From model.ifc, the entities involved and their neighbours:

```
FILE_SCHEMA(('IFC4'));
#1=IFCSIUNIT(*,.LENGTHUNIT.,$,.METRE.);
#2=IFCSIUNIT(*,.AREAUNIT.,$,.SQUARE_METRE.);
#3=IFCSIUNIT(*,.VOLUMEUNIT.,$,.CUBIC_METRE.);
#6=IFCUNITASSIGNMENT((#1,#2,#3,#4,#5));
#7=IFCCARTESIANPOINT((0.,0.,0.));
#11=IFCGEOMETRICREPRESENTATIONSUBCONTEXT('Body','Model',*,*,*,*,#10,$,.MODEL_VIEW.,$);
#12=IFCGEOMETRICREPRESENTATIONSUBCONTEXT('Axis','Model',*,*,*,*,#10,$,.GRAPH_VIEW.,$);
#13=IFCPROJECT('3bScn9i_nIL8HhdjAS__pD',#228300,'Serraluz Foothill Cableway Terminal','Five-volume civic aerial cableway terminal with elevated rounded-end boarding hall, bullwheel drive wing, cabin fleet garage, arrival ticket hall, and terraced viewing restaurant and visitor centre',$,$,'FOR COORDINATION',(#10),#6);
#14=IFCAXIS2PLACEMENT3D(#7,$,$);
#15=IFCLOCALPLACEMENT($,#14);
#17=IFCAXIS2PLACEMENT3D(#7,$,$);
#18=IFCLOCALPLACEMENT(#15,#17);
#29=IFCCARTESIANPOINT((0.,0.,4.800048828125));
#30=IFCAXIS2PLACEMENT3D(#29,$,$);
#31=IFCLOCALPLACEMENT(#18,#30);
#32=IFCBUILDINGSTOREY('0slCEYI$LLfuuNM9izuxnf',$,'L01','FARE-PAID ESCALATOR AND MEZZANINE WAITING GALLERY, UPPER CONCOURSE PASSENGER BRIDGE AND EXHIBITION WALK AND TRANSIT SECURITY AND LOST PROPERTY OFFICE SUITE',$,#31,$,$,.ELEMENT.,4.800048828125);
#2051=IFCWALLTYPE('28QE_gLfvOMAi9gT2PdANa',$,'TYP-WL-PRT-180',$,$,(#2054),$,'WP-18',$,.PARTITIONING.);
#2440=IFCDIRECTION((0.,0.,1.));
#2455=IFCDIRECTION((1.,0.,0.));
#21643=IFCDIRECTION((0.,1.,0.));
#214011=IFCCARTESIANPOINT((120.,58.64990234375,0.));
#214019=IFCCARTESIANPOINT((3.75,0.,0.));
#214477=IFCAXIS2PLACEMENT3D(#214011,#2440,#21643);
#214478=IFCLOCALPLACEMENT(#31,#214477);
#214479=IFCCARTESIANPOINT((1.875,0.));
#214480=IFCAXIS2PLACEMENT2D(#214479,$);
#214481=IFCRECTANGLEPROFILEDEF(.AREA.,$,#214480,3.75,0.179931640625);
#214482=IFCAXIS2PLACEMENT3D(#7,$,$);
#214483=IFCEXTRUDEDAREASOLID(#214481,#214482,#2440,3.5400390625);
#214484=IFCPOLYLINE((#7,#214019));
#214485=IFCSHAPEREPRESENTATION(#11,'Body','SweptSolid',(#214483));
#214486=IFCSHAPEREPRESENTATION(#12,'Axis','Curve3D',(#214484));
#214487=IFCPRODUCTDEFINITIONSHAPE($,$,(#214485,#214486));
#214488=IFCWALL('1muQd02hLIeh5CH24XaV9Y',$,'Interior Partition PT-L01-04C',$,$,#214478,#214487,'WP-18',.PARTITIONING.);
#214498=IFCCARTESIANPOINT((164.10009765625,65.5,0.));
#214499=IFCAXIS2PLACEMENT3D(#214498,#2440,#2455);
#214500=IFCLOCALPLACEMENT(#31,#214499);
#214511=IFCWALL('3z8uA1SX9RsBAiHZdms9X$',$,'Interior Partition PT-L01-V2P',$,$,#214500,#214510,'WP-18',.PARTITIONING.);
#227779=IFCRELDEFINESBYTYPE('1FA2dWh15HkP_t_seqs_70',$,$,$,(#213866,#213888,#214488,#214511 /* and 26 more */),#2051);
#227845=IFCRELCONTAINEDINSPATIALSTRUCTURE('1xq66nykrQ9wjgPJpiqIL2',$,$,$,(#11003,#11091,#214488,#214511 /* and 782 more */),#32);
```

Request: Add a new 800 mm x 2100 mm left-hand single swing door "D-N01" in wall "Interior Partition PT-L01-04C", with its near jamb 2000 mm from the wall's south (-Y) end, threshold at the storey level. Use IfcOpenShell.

```python
import numpy as np
import ifcopenshell
import ifcopenshell.api.feature
import ifcopenshell.api.geometry
import ifcopenshell.api.root
import ifcopenshell.api.spatial
import ifcopenshell.geom
import ifcopenshell.util.element
import ifcopenshell.util.placement
import ifcopenshell.util.representation
import ifcopenshell.util.shape
import ifcopenshell.util.unit

model = ifcopenshell.open("model.ifc")
unit_scale = ifcopenshell.util.unit.calculate_unit_scale(model)
settings = ifcopenshell.geom.settings()


def volume(element):
    """Net volume in cubic metres, openings subtracted."""
    shape = ifcopenshell.geom.create_shape(settings, element)
    return ifcopenshell.util.shape.get_volume(shape.geometry)


wall = model.by_id(214488)
storey = ifcopenshell.util.element.get_container(wall, ifc_class="IfcBuildingStorey")
context = ifcopenshell.util.representation.get_context(model, "Model", "Body", "MODEL_VIEW")
before = volume(wall)

width, height, from_end, sill = 0.8, 2.1, 2, 0.0  # metres

# The wall runs along its own X axis, and the end named is its -X end.
wall_shape = ifcopenshell.geom.create_shape(settings, wall)
x, y, z = ifcopenshell.util.shape.get_vertices(wall_shape.geometry).T
start = x.min() + from_end
face, thickness = float(y.min()), float(y.max() - y.min())
wall_matrix = ifcopenshell.util.placement.get_local_placement(wall.ObjectPlacement)
level = ifcopenshell.util.placement.get_local_placement(storey.ObjectPlacement)[2, 3]


def in_wall(x, y):
    """Placement at x, y metres in the wall's axes, at sill height."""
    matrix = wall_matrix.copy()
    matrix[:, 3] = wall_matrix @ np.array([x / unit_scale, y / unit_scale, 0.0, 1.0])
    matrix[2, 3] = level + sill / unit_scale
    return matrix


# Opening: a box that overshoots both wall faces by 50 mm.
opening = ifcopenshell.api.root.create_entity(model, ifc_class="IfcOpeningElement", predefined_type="OPENING")
box = ifcopenshell.api.geometry.add_wall_representation(
    model, context=context, length=width, height=height, thickness=thickness + 0.1
)
ifcopenshell.api.geometry.assign_representation(model, product=opening, representation=box)
ifcopenshell.api.geometry.edit_object_placement(model, product=opening, matrix=in_wall(start, face - 0.05), is_si=False)
ifcopenshell.api.feature.add_feature(model, feature=opening, element=wall)

door = ifcopenshell.api.root.create_entity(model, ifc_class="IfcDoor", name="D-N01", predefined_type="DOOR")
door.OverallWidth, door.OverallHeight = width / unit_scale, height / unit_scale
door.OperationType = "SINGLE_SWING_LEFT"
body = ifcopenshell.api.geometry.add_door_representation(
    model,
    context=context,
    overall_width=door.OverallWidth,
    overall_height=door.OverallHeight,
    operation_type="SINGLE_SWING_LEFT",
    lining_properties={"LiningDepth": thickness / unit_scale, "ThresholdDepth": thickness / unit_scale},
)
ifcopenshell.api.geometry.assign_representation(model, product=door, representation=body)
ifcopenshell.api.spatial.assign_container(model, products=[door], relating_structure=storey)
ifcopenshell.api.feature.add_filling(model, opening=opening, element=door)

# The lining spans the wall, so the door starts at the wall face.
ifcopenshell.api.geometry.edit_object_placement(model, product=door, matrix=in_wall(start, face), is_si=False)

after = volume(wall)

print(f"wall volume {before:.3f} -> {after:.3f} m3")

model.write("model_edited.ifc")
```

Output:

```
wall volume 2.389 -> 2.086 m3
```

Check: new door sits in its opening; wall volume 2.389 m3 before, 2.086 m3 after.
